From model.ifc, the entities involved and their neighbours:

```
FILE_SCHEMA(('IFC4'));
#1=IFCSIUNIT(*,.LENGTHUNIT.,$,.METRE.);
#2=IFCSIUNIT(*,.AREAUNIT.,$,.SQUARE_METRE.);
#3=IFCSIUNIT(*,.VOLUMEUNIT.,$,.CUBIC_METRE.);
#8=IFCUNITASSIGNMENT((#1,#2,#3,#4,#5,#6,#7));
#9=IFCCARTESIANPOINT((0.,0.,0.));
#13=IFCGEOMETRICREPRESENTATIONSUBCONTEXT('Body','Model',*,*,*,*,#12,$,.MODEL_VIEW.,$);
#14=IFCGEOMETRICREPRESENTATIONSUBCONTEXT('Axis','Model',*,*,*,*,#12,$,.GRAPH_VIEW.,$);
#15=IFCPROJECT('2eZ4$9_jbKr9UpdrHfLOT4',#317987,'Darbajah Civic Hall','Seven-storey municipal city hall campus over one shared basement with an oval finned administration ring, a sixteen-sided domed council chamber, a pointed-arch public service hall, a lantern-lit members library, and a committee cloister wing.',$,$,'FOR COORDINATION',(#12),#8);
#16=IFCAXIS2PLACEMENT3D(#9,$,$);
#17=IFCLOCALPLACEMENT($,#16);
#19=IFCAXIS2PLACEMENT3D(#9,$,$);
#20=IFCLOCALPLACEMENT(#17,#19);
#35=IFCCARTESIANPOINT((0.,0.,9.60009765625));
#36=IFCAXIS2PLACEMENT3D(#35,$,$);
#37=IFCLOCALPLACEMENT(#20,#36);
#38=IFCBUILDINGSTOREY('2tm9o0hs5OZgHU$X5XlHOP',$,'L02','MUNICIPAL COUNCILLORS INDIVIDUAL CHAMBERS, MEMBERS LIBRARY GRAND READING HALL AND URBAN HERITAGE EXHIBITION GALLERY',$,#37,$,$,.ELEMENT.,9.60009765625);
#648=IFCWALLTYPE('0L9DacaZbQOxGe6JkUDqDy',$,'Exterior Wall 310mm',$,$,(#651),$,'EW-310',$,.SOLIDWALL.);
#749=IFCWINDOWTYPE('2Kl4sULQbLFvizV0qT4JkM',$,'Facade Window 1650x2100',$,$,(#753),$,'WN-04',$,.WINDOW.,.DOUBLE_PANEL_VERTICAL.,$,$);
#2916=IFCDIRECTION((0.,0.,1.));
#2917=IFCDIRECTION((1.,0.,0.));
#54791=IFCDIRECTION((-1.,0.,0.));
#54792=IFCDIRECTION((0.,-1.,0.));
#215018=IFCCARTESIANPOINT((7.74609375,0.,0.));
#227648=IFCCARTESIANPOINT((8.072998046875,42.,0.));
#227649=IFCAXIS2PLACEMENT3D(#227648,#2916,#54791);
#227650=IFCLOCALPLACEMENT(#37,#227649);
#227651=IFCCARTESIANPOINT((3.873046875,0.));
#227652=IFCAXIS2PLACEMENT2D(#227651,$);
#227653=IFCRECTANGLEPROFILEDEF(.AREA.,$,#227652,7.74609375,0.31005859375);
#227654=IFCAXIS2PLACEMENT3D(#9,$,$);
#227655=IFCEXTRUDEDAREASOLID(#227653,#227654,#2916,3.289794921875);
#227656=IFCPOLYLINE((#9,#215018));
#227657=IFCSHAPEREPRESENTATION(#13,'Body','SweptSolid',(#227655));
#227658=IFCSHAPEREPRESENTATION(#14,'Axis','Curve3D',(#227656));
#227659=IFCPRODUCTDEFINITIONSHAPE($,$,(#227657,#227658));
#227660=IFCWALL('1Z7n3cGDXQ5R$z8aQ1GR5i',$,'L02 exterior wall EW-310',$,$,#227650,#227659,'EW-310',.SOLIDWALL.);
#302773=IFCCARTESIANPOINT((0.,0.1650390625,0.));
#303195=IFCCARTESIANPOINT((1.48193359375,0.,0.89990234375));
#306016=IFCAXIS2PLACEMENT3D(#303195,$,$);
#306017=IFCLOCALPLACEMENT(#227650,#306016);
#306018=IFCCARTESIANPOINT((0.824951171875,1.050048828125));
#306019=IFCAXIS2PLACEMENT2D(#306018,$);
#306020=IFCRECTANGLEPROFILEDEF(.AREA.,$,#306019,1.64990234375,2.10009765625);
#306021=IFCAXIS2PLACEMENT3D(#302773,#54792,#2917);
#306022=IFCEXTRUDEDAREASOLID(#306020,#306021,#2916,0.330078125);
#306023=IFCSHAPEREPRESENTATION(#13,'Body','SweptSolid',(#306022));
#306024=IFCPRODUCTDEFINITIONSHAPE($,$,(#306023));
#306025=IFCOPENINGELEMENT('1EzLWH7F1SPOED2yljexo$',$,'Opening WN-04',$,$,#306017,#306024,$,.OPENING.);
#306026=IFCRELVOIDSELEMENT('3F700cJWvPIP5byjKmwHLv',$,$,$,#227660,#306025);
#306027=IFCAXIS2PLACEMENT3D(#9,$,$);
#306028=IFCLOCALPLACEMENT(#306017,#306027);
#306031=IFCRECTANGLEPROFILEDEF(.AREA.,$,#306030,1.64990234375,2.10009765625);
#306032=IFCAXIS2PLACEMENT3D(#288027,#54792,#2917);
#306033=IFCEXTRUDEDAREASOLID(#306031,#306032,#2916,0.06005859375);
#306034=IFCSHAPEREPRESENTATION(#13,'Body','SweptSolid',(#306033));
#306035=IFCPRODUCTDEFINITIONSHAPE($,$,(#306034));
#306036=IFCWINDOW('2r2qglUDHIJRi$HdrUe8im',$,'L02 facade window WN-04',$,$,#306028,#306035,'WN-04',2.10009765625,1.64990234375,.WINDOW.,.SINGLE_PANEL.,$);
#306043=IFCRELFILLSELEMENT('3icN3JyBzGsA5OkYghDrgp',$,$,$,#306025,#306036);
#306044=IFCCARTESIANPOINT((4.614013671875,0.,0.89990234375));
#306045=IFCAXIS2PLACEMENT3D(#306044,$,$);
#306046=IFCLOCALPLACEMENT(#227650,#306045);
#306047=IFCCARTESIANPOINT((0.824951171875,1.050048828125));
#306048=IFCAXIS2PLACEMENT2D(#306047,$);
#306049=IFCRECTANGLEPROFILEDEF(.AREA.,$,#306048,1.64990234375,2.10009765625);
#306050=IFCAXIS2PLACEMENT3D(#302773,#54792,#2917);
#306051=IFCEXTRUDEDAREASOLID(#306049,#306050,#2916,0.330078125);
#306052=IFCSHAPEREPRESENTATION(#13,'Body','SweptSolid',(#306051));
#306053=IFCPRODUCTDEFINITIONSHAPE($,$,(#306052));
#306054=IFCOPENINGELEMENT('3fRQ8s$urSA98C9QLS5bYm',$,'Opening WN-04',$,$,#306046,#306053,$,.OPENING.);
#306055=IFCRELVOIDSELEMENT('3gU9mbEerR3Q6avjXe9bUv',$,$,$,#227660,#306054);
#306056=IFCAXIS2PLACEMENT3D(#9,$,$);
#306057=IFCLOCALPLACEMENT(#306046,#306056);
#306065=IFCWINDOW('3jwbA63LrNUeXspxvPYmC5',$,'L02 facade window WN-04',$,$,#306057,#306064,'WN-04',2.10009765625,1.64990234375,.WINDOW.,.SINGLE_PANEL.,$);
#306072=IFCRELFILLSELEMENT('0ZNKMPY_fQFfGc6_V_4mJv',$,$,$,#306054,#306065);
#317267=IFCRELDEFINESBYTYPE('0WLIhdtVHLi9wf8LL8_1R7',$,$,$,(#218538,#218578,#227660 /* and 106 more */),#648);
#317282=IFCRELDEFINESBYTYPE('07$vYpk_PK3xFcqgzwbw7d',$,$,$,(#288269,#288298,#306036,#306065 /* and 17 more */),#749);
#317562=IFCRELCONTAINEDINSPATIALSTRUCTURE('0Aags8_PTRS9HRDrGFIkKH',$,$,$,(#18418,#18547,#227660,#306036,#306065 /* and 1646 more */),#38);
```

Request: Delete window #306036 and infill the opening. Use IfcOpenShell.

```python
import ifcopenshell
import ifcopenshell.api.feature
import ifcopenshell.api.root
import ifcopenshell.geom
import ifcopenshell.util.shape

model = ifcopenshell.open("model.ifc")
settings = ifcopenshell.geom.settings()


def volume(element):
    """Net volume in cubic metres, openings subtracted."""
    shape = ifcopenshell.geom.create_shape(settings, element)
    return ifcopenshell.util.shape.get_volume(shape.geometry)


window = model.by_guid("2r2qglUDHIJRi$HdrUe8im")
opening = window.FillsVoids[0].RelatingOpeningElement
wall = opening.VoidsElements[0].RelatingBuildingElement
before = volume(wall)

ifcopenshell.api.root.remove_product(model, product=window)
ifcopenshell.api.feature.remove_feature(model, feature=opening)

after = volume(wall)

print(f"wall volume {before:.3f} -> {after:.3f} m3")

model.write("model-out.ifc")
```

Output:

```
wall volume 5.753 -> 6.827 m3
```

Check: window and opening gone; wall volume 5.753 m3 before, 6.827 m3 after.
